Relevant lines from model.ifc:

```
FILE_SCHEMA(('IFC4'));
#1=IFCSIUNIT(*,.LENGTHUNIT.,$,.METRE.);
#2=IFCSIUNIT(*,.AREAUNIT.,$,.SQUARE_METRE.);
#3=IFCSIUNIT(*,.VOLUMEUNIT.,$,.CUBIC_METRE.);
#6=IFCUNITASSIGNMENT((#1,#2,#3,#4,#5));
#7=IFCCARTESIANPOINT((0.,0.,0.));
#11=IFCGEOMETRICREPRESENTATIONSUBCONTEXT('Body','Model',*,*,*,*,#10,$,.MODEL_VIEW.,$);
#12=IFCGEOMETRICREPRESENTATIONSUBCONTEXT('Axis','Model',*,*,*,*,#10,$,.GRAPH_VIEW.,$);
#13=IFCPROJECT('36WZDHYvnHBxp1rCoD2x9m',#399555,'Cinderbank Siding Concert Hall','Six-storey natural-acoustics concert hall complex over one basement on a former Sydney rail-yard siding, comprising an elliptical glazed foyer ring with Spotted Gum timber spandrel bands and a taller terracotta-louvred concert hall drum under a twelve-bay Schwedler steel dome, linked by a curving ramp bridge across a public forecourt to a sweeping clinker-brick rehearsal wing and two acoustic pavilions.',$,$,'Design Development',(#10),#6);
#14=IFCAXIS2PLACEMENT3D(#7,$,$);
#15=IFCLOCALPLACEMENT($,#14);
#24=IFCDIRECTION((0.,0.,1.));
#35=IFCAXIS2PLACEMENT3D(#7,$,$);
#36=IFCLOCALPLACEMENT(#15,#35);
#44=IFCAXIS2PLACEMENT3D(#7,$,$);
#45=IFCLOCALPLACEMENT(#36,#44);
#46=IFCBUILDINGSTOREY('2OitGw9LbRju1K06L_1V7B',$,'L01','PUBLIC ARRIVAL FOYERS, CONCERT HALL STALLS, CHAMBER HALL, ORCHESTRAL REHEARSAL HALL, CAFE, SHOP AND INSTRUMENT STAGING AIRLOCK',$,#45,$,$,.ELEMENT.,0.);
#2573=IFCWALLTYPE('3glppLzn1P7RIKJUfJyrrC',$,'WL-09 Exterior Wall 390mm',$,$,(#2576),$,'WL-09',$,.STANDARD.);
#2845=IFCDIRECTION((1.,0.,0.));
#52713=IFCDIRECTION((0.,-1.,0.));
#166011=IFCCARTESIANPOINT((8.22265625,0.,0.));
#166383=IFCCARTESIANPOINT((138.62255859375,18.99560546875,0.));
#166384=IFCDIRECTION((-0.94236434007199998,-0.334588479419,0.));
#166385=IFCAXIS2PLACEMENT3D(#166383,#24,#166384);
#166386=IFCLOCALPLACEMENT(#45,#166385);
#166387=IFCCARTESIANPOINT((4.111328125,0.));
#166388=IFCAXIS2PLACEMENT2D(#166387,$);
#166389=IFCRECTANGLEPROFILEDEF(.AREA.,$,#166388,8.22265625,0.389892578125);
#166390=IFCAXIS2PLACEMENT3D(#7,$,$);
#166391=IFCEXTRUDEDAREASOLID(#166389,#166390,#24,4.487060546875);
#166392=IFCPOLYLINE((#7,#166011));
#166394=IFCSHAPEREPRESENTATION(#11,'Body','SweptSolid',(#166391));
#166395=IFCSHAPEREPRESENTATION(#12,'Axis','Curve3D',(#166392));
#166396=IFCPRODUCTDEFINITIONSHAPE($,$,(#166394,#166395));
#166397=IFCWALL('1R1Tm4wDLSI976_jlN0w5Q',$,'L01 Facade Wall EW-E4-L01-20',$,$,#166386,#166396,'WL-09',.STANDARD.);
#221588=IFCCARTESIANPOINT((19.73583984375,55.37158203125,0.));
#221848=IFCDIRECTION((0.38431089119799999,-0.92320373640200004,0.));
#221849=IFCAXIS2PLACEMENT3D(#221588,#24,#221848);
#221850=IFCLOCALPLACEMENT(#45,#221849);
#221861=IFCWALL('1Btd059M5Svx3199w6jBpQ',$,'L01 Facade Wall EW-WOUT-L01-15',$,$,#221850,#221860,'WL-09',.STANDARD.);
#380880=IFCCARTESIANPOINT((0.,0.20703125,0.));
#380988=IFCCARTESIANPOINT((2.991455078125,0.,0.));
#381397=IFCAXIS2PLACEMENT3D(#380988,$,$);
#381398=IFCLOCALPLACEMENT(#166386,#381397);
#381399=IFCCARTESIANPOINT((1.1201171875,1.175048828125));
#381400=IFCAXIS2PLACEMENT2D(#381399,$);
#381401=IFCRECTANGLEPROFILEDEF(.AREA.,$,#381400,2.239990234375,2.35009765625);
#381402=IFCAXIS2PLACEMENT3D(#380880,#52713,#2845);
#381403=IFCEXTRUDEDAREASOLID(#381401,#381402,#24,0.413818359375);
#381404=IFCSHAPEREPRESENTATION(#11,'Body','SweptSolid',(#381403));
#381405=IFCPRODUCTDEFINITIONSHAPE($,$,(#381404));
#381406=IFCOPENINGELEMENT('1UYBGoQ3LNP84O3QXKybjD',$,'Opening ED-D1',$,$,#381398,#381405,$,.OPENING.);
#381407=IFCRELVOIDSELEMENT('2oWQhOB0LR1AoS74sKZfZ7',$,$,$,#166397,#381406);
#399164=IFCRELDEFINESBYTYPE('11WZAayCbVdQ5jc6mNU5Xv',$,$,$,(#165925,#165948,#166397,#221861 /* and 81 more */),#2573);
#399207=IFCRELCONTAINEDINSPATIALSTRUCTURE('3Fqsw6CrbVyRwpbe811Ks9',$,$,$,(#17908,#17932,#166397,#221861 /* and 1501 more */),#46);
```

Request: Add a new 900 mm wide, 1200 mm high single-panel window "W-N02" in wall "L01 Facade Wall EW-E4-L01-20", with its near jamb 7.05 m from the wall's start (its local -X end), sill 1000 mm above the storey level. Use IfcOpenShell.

```python
import numpy as np
import ifcopenshell
import ifcopenshell.api.feature
import ifcopenshell.api.geometry
import ifcopenshell.api.root
import ifcopenshell.api.spatial
import ifcopenshell.geom
import ifcopenshell.util.element
import ifcopenshell.util.placement
import ifcopenshell.util.representation
import ifcopenshell.util.shape
import ifcopenshell.util.unit

model = ifcopenshell.open("model.ifc")
unit_scale = ifcopenshell.util.unit.calculate_unit_scale(model)
settings = ifcopenshell.geom.settings()


def volume(element):
    """Net volume in cubic metres, openings subtracted."""
    shape = ifcopenshell.geom.create_shape(settings, element)
    return ifcopenshell.util.shape.get_volume(shape.geometry)


wall = model.by_guid("1R1Tm4wDLSI976_jlN0w5Q")
storey = ifcopenshell.util.element.get_container(wall, ifc_class="IfcBuildingStorey")
context = ifcopenshell.util.representation.get_context(model, "Model", "Body", "MODEL_VIEW")
before = volume(wall)

width, height, from_end, sill = 0.9, 1.2, 7.05, 1  # metres

# The wall runs along its own X axis, and the end named is its -X end.
wall_shape = ifcopenshell.geom.create_shape(settings, wall)
x, y, z = ifcopenshell.util.shape.get_vertices(wall_shape.geometry).T
start = x.min() + from_end
face, thickness = float(y.min()), float(y.max() - y.min())
wall_matrix = ifcopenshell.util.placement.get_local_placement(wall.ObjectPlacement)
level = ifcopenshell.util.placement.get_local_placement(storey.ObjectPlacement)[2, 3]


def in_wall(x, y):
    """Placement at x, y metres in the wall's axes, at sill height."""
    matrix = wall_matrix.copy()
    matrix[:, 3] = wall_matrix @ np.array([x / unit_scale, y / unit_scale, 0.0, 1.0])
    matrix[2, 3] = level + sill / unit_scale
    return matrix


# Opening: a box that overshoots both wall faces by 50 mm.
opening = ifcopenshell.api.root.create_entity(model, ifc_class="IfcOpeningElement", predefined_type="OPENING")
box = ifcopenshell.api.geometry.add_wall_representation(
    model, context=context, length=width, height=height, thickness=thickness + 0.1
)
ifcopenshell.api.geometry.assign_representation(model, product=opening, representation=box)
ifcopenshell.api.geometry.edit_object_placement(model, product=opening, matrix=in_wall(start, face - 0.05), is_si=False)
ifcopenshell.api.feature.add_feature(model, feature=opening, element=wall)

window = ifcopenshell.api.root.create_entity(model, ifc_class="IfcWindow", name="W-N02", predefined_type="WINDOW")
window.OverallWidth, window.OverallHeight = width / unit_scale, height / unit_scale
window.PartitioningType = "SINGLE_PANEL"
body = ifcopenshell.api.geometry.add_window_representation(
    model,
    context=context,
    overall_width=window.OverallWidth,
    overall_height=window.OverallHeight,
    partition_type="SINGLE_PANEL",
)
ifcopenshell.api.geometry.assign_representation(model, product=window, representation=body)
ifcopenshell.api.spatial.assign_container(model, products=[window], relating_structure=storey)
ifcopenshell.api.feature.add_filling(model, opening=opening, element=window)

# Centre the window in the wall's thickness.
ifcopenshell.api.geometry.edit_object_placement(model, product=window, matrix=in_wall(start, face), is_si=False)
window_shape = ifcopenshell.geom.create_shape(settings, window)
depth = ifcopenshell.util.shape.get_vertices(window_shape.geometry)[:, 1]
offset = face + thickness / 2 - (depth.min() + depth.max()) / 2
ifcopenshell.api.geometry.edit_object_placement(model, product=window, matrix=in_wall(start, offset), is_si=False)

after = volume(wall)

print(f"wall volume {before:.3f} -> {after:.3f} m3")

model.write("model_rev.ifc")
```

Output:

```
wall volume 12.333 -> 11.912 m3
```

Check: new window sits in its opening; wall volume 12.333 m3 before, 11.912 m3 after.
